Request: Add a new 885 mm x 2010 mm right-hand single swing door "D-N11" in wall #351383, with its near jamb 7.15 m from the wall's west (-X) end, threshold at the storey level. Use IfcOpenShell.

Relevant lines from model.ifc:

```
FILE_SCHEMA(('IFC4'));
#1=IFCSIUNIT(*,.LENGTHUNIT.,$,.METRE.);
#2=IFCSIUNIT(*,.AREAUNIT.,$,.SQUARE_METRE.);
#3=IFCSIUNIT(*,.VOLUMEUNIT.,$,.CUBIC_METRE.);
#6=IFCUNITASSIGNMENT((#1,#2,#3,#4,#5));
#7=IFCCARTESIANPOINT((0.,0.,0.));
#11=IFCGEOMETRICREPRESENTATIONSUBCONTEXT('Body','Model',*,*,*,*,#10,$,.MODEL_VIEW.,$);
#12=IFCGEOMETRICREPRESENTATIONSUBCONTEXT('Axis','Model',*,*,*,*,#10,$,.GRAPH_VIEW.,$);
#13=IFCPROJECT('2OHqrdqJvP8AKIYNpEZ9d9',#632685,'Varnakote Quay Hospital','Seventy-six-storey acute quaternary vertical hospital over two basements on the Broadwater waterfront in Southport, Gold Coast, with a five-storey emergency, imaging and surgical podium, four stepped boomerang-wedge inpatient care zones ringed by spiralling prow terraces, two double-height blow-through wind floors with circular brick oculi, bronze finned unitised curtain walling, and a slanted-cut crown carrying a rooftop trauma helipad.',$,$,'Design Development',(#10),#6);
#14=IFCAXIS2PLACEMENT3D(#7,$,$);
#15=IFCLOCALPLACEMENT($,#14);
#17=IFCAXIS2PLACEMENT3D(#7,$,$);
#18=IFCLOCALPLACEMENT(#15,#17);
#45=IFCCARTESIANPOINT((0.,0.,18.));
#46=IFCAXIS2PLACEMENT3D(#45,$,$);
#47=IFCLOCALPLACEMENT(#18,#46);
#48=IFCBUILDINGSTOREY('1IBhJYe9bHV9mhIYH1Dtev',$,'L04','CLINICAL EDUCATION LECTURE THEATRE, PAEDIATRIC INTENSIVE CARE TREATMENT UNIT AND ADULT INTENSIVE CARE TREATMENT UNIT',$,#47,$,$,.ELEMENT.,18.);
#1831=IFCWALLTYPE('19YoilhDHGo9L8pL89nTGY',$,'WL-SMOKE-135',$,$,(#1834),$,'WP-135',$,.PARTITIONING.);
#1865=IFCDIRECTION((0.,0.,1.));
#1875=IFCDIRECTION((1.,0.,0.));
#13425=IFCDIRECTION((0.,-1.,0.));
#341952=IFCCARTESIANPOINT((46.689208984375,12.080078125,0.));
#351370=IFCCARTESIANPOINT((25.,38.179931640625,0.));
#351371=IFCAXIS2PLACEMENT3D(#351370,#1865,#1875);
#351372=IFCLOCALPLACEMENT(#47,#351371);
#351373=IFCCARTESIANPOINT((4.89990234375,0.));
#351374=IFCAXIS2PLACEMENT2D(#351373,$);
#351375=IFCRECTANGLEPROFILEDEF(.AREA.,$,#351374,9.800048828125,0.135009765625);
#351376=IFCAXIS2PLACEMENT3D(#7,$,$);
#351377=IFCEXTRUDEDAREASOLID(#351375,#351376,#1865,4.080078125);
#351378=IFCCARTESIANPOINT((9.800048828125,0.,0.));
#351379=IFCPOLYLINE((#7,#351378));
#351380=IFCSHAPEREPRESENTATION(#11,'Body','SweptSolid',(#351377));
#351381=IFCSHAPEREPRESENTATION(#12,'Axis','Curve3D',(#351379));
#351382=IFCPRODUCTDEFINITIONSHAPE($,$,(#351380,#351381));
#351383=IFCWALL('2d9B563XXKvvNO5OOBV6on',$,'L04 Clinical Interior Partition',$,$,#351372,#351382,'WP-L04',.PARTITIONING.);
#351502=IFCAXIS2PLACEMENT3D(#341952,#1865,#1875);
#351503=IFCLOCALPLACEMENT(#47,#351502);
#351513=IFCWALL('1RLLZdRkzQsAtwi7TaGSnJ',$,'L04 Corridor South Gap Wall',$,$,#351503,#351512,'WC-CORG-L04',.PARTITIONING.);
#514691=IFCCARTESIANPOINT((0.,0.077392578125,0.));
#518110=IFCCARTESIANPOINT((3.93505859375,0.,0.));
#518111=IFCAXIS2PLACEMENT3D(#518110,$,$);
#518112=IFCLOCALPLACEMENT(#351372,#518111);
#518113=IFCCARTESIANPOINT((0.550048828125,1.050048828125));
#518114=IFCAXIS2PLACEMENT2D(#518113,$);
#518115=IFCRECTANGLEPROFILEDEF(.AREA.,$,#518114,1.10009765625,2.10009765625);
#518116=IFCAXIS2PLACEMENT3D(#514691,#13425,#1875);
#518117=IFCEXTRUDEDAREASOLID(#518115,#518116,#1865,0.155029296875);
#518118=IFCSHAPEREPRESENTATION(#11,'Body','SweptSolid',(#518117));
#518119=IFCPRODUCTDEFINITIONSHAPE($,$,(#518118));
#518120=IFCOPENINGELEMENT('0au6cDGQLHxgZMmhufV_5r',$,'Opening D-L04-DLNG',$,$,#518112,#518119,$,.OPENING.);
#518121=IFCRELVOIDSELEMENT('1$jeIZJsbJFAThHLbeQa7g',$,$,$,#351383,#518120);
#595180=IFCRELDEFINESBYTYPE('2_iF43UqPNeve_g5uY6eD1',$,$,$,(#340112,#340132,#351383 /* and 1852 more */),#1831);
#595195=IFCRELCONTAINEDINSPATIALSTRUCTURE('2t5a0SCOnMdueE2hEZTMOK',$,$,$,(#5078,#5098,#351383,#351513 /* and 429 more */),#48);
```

```python
import numpy as np
import ifcopenshell
import ifcopenshell.api.feature
import ifcopenshell.api.geometry
import ifcopenshell.api.root
import ifcopenshell.api.spatial
import ifcopenshell.geom
import ifcopenshell.util.element
import ifcopenshell.util.placement
import ifcopenshell.util.representation
import ifcopenshell.util.shape
import ifcopenshell.util.unit

model = ifcopenshell.open("model.ifc")
unit_scale = ifcopenshell.util.unit.calculate_unit_scale(model)
settings = ifcopenshell.geom.settings()


def volume(element):
    """Net volume in cubic metres, openings subtracted."""
    shape = ifcopenshell.geom.create_shape(settings, element)
    return ifcopenshell.util.shape.get_volume(shape.geometry)


wall = model.by_id(351383)
storey = ifcopenshell.util.element.get_container(wall, ifc_class="IfcBuildingStorey")
context = ifcopenshell.util.representation.get_context(model, "Model", "Body", "MODEL_VIEW")
before = volume(wall)

width, height, from_end, sill = 0.885, 2.01, 7.15, 0.0  # metres

# The wall runs along its own X axis, and the end named is its -X end.
wall_shape = ifcopenshell.geom.create_shape(settings, wall)
x, y, z = ifcopenshell.util.shape.get_vertices(wall_shape.geometry).T
start = x.min() + from_end
face, thickness = float(y.min()), float(y.max() - y.min())
wall_matrix = ifcopenshell.util.placement.get_local_placement(wall.ObjectPlacement)
level = ifcopenshell.util.placement.get_local_placement(storey.ObjectPlacement)[2, 3]


def in_wall(x, y):
    """Placement at x, y metres in the wall's axes, at sill height."""
    matrix = wall_matrix.copy()
    matrix[:, 3] = wall_matrix @ np.array([x / unit_scale, y / unit_scale, 0.0, 1.0])
    matrix[2, 3] = level + sill / unit_scale
    return matrix


# Opening: a box that overshoots both wall faces by 50 mm.
opening = ifcopenshell.api.root.create_entity(model, ifc_class="IfcOpeningElement", predefined_type="OPENING")
box = ifcopenshell.api.geometry.add_wall_representation(
    model, context=context, length=width, height=height, thickness=thickness + 0.1
)
ifcopenshell.api.geometry.assign_representation(model, product=opening, representation=box)
ifcopenshell.api.geometry.edit_object_placement(model, product=opening, matrix=in_wall(start, face - 0.05), is_si=False)
ifcopenshell.api.feature.add_feature(model, feature=opening, element=wall)

door = ifcopenshell.api.root.create_entity(model, ifc_class="IfcDoor", name="D-N11", predefined_type="DOOR")
door.OverallWidth, door.OverallHeight = width / unit_scale, height / unit_scale
door.OperationType = "SINGLE_SWING_RIGHT"
body = ifcopenshell.api.geometry.add_door_representation(
    model,
    context=context,
    overall_width=door.OverallWidth,
    overall_height=door.OverallHeight,
    operation_type="SINGLE_SWING_RIGHT",
    lining_properties={"LiningDepth": thickness / unit_scale, "ThresholdDepth": thickness / unit_scale},
)
ifcopenshell.api.geometry.assign_representation(model, product=door, representation=body)
ifcopenshell.api.spatial.assign_container(model, products=[door], relating_structure=storey)
ifcopenshell.api.feature.add_filling(model, opening=opening, element=door)

# The lining spans the wall, so the door starts at the wall face.
ifcopenshell.api.geometry.edit_object_placement(model, product=door, matrix=in_wall(start, face), is_si=False)

after = volume(wall)

print(f"wall volume {before:.3f} -> {after:.3f} m3")

model.write("model-out.ifc")
```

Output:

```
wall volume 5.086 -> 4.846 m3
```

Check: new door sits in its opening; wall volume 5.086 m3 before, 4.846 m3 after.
